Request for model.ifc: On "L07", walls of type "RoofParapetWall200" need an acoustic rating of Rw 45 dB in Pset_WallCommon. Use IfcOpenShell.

First a look at what the model holds.

```python
import ifcopenshell
import ifcopenshell.util.element

model = ifcopenshell.open("model.ifc")
print(model.schema)
storey = next(s for s in model.by_type("IfcBuildingStorey") if s.Name == "L07")
walls = [e for e in ifcopenshell.util.element.get_decomposition(storey) if e.is_a("IfcWall")]
seen = {}
for e in walls:
    element_type = ifcopenshell.util.element.get_type(e)
    key = (element_type.Name if element_type != e and element_type else None, ifcopenshell.util.element.get_pset(e, "Pset_WallCommon", "AcousticRating"))
    seen[key] = seen.get(key, 0) + 1
for (name, value), count in sorted(seen.items(), key=str):
    print(count, "x", name, "|", value)
```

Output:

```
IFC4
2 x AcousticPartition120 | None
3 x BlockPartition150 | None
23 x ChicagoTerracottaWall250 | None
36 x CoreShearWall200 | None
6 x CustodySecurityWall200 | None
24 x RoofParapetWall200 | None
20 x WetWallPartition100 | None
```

```python
import ifcopenshell
import ifcopenshell.api.pset
import ifcopenshell.util.element

model = ifcopenshell.open("model.ifc")

storey = next(s for s in model.by_type("IfcBuildingStorey") if s.Name == "L07")
walls = [e for e in ifcopenshell.util.element.get_decomposition(storey) if e.is_a("IfcWall")]

count = 0
for e in walls:
    element_type = ifcopenshell.util.element.get_type(e)
    if element_type in (None, e) or element_type.Name != "RoofParapetWall200":
        continue
    # add_pset returns the element's existing set when there is one.
    pset = ifcopenshell.api.pset.add_pset(model, product=e, name="Pset_WallCommon")
    ifcopenshell.api.pset.edit_pset(model, pset=pset, properties={"AcousticRating": "Rw 45 dB"})
    count += 1

print(count, "walls updated")

model.write("model_updated.ifc")
```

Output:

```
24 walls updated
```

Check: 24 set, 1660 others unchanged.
